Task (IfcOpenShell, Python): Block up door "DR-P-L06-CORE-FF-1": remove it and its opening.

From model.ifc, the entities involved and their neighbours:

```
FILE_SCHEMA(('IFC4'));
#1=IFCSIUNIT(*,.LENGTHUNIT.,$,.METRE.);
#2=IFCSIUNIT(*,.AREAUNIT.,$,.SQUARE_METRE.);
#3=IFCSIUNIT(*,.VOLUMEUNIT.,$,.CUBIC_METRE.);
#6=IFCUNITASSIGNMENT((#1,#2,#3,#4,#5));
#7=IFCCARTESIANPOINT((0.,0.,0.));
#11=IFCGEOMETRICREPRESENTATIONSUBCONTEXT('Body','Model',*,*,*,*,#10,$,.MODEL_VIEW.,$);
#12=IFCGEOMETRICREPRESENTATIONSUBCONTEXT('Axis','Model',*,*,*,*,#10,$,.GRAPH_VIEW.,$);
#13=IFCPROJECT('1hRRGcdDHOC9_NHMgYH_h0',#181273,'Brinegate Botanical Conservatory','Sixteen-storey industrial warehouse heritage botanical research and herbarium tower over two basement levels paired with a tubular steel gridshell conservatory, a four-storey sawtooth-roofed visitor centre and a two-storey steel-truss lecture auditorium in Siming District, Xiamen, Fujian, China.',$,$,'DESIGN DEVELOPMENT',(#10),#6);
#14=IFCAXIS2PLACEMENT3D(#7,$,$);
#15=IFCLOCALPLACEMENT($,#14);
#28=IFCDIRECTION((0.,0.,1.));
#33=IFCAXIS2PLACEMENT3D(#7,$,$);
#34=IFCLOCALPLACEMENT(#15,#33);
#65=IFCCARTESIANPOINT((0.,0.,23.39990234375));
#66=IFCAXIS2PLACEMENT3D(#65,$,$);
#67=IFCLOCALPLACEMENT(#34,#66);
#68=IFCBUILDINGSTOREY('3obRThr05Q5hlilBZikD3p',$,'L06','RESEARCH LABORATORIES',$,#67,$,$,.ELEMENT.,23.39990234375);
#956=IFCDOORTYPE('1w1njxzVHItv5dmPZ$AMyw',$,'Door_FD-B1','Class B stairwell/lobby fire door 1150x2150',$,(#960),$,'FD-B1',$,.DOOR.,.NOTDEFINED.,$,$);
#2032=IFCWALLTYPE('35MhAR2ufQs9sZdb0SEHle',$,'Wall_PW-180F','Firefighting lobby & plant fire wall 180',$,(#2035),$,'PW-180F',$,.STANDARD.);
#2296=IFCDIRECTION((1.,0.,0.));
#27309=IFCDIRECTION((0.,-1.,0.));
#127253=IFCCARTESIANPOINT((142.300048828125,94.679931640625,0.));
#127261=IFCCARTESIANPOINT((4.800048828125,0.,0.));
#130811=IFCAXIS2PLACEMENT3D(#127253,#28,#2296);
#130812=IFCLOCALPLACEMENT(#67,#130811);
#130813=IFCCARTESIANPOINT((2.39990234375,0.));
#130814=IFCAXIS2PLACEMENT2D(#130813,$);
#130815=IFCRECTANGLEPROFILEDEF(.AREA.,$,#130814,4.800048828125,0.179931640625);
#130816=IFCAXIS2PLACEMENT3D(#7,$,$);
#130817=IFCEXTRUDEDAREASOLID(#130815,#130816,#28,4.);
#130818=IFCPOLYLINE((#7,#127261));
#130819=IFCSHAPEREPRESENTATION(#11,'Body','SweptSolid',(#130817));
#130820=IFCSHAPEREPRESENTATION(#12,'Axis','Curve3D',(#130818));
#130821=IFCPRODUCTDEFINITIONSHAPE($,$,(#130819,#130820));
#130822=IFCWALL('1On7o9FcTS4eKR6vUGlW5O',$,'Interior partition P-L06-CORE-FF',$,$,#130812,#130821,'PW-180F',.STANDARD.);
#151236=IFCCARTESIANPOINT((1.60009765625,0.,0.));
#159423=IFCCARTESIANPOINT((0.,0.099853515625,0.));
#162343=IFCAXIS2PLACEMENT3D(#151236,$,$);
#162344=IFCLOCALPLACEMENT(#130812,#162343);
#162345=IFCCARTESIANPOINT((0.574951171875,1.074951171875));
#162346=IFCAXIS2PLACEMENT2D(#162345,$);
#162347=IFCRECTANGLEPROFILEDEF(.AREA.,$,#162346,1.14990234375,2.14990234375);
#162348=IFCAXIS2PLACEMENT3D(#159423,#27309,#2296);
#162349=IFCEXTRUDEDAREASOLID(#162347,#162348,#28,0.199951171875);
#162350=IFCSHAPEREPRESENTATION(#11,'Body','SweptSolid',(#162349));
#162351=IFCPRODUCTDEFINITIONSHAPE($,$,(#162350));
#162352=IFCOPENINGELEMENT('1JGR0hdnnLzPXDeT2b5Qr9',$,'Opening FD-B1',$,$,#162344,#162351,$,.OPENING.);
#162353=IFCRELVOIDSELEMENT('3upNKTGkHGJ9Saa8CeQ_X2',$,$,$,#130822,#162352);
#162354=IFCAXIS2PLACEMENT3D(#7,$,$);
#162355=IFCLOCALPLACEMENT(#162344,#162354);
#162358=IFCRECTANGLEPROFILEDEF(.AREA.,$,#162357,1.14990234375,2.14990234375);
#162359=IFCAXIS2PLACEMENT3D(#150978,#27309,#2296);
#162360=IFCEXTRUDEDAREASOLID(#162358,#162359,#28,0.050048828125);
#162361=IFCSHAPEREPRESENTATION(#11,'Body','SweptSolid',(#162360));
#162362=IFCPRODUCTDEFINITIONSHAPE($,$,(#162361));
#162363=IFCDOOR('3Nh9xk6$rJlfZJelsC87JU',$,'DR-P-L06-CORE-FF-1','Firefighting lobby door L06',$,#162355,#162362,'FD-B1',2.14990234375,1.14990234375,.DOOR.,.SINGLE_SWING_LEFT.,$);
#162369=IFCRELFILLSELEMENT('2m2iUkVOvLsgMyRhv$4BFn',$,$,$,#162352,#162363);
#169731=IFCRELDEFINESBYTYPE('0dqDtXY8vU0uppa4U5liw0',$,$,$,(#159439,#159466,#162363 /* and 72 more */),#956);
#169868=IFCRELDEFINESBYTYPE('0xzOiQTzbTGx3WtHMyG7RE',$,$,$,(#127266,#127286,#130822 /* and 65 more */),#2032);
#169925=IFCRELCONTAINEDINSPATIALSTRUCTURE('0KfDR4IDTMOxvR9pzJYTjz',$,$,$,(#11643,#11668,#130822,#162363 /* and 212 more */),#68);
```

```python
import ifcopenshell
import ifcopenshell.api.feature
import ifcopenshell.api.root
import ifcopenshell.geom
import ifcopenshell.util.shape

model = ifcopenshell.open("model.ifc")
settings = ifcopenshell.geom.settings()


def volume(element):
    """Net volume in cubic metres, openings subtracted."""
    shape = ifcopenshell.geom.create_shape(settings, element)
    return ifcopenshell.util.shape.get_volume(shape.geometry)


door = model.by_id(162363)
opening = door.FillsVoids[0].RelatingOpeningElement
wall = opening.VoidsElements[0].RelatingBuildingElement
before = volume(wall)

ifcopenshell.api.root.remove_product(model, product=door)
ifcopenshell.api.feature.remove_feature(model, feature=opening)

after = volume(wall)

print(f"wall volume {before:.3f} -> {after:.3f} m3")

model.write("model-out.ifc")
```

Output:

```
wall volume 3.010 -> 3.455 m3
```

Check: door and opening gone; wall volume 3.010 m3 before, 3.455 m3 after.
